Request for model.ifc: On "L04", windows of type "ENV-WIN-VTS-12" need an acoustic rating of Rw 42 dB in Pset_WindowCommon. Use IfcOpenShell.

First a look at what the model holds.

```python
import ifcopenshell
import ifcopenshell.util.element

model = ifcopenshell.open("model.ifc")
print(model.schema)
storey = next(s for s in model.by_type("IfcBuildingStorey") if s.Name == "L04")
windows = [e for e in ifcopenshell.util.element.get_decomposition(storey) if e.is_a("IfcWindow")]
seen = {}
for e in windows:
    element_type = ifcopenshell.util.element.get_type(e)
    key = (element_type.Name if element_type != e and element_type else None, ifcopenshell.util.element.get_pset(e, "Pset_WindowCommon", "AcousticRating"))
    seen[key] = seen.get(key, 0) + 1
for (name, value), count in sorted(seen.items(), key=str):
    print(count, "x", name, "|", value)
```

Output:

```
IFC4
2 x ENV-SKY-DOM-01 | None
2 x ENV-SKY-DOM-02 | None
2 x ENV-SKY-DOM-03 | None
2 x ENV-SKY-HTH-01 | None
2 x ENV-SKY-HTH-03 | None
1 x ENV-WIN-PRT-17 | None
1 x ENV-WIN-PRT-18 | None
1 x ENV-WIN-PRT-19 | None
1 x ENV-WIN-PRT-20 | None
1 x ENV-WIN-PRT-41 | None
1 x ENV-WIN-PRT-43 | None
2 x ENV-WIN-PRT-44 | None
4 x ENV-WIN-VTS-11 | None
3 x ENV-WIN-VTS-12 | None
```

```python
import ifcopenshell
import ifcopenshell.api.pset
import ifcopenshell.util.element

model = ifcopenshell.open("model.ifc")

storey = next(s for s in model.by_type("IfcBuildingStorey") if s.Name == "L04")
windows = [e for e in ifcopenshell.util.element.get_decomposition(storey) if e.is_a("IfcWindow")]

count = 0
for e in windows:
    element_type = ifcopenshell.util.element.get_type(e)
    if element_type in (None, e) or element_type.Name != "ENV-WIN-VTS-12":
        continue
    # add_pset returns the element's existing set when there is one.
    pset = ifcopenshell.api.pset.add_pset(model, product=e, name="Pset_WindowCommon")
    ifcopenshell.api.pset.edit_pset(model, pset=pset, properties={"AcousticRating": "Rw 42 dB"})
    count += 1

print(count, "windows updated")

model.write("model_rev.ifc")
```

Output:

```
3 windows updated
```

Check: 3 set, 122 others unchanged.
